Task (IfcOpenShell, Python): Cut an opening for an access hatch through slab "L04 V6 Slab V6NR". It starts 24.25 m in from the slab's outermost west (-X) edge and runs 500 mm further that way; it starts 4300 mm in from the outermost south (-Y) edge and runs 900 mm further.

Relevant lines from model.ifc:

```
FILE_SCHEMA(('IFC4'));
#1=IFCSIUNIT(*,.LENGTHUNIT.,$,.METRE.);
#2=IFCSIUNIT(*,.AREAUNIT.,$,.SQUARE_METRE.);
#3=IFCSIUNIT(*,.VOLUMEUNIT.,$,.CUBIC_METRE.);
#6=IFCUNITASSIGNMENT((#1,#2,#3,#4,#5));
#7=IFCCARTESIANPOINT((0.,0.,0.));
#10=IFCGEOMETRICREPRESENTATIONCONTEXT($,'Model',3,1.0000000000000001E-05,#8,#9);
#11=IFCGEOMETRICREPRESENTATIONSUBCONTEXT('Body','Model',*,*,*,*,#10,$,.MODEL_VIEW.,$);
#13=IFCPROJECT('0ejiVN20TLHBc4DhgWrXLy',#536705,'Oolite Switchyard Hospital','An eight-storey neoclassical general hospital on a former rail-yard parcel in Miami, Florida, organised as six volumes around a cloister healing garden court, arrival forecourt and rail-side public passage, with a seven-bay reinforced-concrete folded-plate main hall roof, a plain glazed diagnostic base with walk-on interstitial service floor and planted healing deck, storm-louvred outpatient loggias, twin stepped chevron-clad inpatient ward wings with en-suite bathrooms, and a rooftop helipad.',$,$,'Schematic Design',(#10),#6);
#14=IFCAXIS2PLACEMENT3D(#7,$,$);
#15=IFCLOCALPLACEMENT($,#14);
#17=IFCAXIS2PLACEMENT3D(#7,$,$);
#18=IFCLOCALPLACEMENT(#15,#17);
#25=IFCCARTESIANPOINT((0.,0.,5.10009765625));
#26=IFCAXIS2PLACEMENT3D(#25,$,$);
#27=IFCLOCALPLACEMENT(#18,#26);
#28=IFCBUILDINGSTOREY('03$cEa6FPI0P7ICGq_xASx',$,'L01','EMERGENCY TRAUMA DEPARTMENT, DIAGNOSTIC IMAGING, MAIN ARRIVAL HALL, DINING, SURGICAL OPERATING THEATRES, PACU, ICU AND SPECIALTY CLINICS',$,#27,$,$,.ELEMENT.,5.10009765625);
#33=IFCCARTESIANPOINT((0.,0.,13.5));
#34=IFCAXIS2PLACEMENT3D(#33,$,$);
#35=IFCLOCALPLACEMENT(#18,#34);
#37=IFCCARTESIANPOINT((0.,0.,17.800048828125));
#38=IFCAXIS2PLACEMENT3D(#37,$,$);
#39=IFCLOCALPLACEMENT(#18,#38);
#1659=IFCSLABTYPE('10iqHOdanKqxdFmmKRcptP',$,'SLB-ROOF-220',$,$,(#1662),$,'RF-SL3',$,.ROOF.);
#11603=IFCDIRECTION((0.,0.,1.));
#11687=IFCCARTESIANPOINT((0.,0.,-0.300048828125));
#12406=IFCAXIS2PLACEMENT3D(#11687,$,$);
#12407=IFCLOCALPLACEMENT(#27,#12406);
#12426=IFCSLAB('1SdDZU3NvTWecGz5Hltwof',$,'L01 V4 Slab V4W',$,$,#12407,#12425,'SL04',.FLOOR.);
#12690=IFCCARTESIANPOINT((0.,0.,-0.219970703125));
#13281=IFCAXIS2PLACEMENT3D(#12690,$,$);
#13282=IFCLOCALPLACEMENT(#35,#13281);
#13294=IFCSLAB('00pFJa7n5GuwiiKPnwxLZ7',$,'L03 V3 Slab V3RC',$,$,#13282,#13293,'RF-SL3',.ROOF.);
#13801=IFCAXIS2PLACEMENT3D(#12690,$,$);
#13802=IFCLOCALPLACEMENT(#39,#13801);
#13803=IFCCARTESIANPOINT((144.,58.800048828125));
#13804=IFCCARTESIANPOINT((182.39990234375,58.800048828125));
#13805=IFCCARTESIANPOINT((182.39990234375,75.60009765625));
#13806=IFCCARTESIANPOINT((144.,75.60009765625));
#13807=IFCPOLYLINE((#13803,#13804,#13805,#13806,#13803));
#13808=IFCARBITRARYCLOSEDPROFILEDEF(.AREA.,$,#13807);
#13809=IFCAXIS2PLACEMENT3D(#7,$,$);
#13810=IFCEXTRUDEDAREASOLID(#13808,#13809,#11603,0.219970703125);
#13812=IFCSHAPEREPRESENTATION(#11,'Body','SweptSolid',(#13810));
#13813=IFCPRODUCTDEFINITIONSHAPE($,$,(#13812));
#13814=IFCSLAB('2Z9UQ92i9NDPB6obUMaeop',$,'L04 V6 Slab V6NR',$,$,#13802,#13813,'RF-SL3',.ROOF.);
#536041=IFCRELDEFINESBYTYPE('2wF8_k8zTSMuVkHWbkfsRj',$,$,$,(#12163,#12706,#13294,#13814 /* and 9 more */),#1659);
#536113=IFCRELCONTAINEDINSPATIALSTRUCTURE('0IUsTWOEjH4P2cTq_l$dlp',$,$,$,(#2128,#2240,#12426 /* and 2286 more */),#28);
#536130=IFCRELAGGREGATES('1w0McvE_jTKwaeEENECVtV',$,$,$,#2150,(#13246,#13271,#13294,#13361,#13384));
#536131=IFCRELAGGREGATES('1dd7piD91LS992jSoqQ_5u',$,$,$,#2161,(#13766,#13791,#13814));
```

```python
import numpy as np
import ifcopenshell
import ifcopenshell.api.feature
import ifcopenshell.api.geometry
import ifcopenshell.api.root
import ifcopenshell.geom
import ifcopenshell.util.placement
import ifcopenshell.util.representation
import ifcopenshell.util.shape
import ifcopenshell.util.unit

model = ifcopenshell.open("model.ifc")
unit_scale = ifcopenshell.util.unit.calculate_unit_scale(model)
settings = ifcopenshell.geom.settings()


def volume(element):
    """Net volume in cubic metres, openings subtracted."""
    shape = ifcopenshell.geom.create_shape(settings, element)
    return ifcopenshell.util.shape.get_volume(shape.geometry)


slab = model.by_guid("2Z9UQ92i9NDPB6obUMaeop")
before = volume(slab)

# Extent in the slab's own axes, in metres. The edges named are its -X and -Y sides.
slab_shape = ifcopenshell.geom.create_shape(settings, slab)
vertices = ifcopenshell.util.shape.get_vertices(slab_shape.geometry)
x_min, y_min, bottom = vertices.min(axis=0)
top = vertices[:, 2].max()

opening = ifcopenshell.api.root.create_entity(model, ifc_class="IfcOpeningElement", name="Access hatch opening", predefined_type="OPENING")
context = ifcopenshell.util.representation.get_context(model, "Model", "Body", "MODEL_VIEW")
width, depth = 0.5, 0.9
outline = [(0.0, 0.0), (width, 0.0), (width, depth), (0.0, depth), (0.0, 0.0)]
# Overshoot both faces by 50 mm so the cut is clean.
shape = ifcopenshell.api.geometry.add_slab_representation(
    model, context=context, depth=top - bottom + 0.1, polyline=outline
)
ifcopenshell.api.geometry.assign_representation(model, product=opening, representation=shape)

matrix = ifcopenshell.util.placement.get_local_placement(slab.ObjectPlacement)
matrix[:, 3] = matrix @ np.append(np.array([x_min + 24.25, y_min + 4.3, bottom - 0.05]) / unit_scale, 1.0)
ifcopenshell.api.geometry.edit_object_placement(model, product=opening, matrix=matrix, is_si=False)
ifcopenshell.api.feature.add_feature(model, feature=opening, element=slab)

after = volume(slab)

print(f"slab volume {before:.3f} -> {after:.3f} m3")

model.write("model_v2.ifc")
```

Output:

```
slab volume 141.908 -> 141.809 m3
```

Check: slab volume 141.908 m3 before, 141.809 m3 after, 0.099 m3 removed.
